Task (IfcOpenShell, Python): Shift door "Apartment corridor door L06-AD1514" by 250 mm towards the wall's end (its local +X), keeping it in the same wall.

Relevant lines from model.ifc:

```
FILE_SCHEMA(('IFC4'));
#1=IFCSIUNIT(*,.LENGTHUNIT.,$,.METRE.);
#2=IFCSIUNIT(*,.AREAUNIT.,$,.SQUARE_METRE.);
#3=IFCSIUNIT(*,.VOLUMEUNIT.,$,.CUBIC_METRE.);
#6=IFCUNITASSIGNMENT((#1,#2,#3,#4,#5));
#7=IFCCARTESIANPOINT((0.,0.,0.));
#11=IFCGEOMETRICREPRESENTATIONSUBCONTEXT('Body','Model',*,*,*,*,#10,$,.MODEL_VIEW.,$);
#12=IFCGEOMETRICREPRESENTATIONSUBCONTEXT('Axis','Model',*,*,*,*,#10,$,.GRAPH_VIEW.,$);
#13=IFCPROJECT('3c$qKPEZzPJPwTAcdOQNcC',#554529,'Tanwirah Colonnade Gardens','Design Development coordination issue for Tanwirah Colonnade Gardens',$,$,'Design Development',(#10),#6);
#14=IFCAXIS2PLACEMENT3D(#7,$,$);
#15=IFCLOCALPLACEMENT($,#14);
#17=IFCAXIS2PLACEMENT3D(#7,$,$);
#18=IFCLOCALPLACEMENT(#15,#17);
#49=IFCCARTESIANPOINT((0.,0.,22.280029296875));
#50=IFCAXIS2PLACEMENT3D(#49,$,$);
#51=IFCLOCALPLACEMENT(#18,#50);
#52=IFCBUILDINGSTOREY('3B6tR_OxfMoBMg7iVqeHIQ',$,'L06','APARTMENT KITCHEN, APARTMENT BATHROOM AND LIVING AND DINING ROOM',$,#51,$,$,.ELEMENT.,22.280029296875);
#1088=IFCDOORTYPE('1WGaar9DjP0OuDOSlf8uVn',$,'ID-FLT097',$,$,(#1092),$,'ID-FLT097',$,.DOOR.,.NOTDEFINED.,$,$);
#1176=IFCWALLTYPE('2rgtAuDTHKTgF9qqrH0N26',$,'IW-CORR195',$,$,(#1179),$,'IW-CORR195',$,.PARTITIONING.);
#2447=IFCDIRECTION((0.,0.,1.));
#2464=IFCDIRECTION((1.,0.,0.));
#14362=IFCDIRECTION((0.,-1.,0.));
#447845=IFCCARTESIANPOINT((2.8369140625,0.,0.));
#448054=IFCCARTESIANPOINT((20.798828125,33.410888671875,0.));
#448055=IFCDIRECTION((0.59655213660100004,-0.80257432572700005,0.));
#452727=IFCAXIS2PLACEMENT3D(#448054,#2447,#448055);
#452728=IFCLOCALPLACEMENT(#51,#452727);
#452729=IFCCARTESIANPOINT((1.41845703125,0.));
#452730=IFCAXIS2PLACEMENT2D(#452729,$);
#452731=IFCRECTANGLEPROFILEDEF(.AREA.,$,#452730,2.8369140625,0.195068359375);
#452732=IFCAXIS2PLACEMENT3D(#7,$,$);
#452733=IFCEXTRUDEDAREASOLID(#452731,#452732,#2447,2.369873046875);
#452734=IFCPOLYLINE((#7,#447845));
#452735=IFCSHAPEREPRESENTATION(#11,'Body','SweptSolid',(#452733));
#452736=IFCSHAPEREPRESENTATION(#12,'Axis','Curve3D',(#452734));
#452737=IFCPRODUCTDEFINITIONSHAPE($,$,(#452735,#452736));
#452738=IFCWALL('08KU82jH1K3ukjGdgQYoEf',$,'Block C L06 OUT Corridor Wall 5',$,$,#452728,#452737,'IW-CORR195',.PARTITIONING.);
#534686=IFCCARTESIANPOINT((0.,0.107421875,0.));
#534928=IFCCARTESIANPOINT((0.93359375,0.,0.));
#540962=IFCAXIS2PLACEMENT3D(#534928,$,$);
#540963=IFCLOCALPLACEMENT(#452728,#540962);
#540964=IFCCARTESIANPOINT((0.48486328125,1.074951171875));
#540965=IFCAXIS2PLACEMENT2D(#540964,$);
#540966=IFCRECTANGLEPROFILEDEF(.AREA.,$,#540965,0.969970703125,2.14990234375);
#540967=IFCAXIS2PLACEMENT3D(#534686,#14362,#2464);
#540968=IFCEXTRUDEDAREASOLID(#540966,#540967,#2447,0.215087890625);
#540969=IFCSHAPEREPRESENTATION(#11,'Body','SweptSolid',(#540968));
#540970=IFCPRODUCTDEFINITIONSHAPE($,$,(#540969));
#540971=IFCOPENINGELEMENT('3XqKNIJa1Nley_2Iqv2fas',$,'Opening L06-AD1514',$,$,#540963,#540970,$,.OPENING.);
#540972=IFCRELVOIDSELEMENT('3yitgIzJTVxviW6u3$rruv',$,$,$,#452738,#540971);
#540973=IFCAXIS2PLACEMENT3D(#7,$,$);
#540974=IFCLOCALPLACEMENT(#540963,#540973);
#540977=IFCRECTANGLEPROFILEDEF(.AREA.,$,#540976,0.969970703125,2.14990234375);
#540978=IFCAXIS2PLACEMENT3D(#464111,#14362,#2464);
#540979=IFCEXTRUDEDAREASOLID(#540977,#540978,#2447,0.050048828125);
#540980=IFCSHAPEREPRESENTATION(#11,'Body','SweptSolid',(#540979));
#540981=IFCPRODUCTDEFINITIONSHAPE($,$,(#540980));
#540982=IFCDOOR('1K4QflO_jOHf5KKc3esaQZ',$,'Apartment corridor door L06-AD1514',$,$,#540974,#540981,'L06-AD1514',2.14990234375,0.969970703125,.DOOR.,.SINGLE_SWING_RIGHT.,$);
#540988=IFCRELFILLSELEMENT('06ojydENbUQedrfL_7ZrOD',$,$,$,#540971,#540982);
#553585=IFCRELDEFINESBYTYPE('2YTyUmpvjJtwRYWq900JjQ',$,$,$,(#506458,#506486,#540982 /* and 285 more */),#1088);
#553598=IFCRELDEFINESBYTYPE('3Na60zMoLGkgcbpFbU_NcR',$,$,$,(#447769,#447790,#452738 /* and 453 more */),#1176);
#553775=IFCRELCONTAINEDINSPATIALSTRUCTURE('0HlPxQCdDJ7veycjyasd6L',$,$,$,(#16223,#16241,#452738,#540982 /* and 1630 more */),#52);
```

```python
import ifcopenshell
import ifcopenshell.api.geometry
import ifcopenshell.util.placement

model = ifcopenshell.open("model.ifc")

door = model.by_guid("1K4QflO_jOHf5KKc3esaQZ")
opening = door.FillsVoids[0].RelatingOpeningElement
wall = opening.VoidsElements[0].RelatingBuildingElement

wall_matrix = ifcopenshell.util.placement.get_local_placement(wall.ObjectPlacement)
shift = wall_matrix[:3, 0] * 0.25
before = ifcopenshell.util.placement.get_local_placement(door.ObjectPlacement)[:3, 3].copy()

# The door is placed relative to its opening, so it follows when the opening moves.
matrix = ifcopenshell.util.placement.get_local_placement(opening.ObjectPlacement)
matrix[:3, 3] += shift
ifcopenshell.api.geometry.edit_object_placement(
    model, product=opening, matrix=matrix, is_si=False, should_transform_children=True
)

after = ifcopenshell.util.placement.get_local_placement(door.ObjectPlacement)[:3, 3]
print("door moved by", (after - before).round(3) + 0.0)

model.write("model_edited.ifc")
```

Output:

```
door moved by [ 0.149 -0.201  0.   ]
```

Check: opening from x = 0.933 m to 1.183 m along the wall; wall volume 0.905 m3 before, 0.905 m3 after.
